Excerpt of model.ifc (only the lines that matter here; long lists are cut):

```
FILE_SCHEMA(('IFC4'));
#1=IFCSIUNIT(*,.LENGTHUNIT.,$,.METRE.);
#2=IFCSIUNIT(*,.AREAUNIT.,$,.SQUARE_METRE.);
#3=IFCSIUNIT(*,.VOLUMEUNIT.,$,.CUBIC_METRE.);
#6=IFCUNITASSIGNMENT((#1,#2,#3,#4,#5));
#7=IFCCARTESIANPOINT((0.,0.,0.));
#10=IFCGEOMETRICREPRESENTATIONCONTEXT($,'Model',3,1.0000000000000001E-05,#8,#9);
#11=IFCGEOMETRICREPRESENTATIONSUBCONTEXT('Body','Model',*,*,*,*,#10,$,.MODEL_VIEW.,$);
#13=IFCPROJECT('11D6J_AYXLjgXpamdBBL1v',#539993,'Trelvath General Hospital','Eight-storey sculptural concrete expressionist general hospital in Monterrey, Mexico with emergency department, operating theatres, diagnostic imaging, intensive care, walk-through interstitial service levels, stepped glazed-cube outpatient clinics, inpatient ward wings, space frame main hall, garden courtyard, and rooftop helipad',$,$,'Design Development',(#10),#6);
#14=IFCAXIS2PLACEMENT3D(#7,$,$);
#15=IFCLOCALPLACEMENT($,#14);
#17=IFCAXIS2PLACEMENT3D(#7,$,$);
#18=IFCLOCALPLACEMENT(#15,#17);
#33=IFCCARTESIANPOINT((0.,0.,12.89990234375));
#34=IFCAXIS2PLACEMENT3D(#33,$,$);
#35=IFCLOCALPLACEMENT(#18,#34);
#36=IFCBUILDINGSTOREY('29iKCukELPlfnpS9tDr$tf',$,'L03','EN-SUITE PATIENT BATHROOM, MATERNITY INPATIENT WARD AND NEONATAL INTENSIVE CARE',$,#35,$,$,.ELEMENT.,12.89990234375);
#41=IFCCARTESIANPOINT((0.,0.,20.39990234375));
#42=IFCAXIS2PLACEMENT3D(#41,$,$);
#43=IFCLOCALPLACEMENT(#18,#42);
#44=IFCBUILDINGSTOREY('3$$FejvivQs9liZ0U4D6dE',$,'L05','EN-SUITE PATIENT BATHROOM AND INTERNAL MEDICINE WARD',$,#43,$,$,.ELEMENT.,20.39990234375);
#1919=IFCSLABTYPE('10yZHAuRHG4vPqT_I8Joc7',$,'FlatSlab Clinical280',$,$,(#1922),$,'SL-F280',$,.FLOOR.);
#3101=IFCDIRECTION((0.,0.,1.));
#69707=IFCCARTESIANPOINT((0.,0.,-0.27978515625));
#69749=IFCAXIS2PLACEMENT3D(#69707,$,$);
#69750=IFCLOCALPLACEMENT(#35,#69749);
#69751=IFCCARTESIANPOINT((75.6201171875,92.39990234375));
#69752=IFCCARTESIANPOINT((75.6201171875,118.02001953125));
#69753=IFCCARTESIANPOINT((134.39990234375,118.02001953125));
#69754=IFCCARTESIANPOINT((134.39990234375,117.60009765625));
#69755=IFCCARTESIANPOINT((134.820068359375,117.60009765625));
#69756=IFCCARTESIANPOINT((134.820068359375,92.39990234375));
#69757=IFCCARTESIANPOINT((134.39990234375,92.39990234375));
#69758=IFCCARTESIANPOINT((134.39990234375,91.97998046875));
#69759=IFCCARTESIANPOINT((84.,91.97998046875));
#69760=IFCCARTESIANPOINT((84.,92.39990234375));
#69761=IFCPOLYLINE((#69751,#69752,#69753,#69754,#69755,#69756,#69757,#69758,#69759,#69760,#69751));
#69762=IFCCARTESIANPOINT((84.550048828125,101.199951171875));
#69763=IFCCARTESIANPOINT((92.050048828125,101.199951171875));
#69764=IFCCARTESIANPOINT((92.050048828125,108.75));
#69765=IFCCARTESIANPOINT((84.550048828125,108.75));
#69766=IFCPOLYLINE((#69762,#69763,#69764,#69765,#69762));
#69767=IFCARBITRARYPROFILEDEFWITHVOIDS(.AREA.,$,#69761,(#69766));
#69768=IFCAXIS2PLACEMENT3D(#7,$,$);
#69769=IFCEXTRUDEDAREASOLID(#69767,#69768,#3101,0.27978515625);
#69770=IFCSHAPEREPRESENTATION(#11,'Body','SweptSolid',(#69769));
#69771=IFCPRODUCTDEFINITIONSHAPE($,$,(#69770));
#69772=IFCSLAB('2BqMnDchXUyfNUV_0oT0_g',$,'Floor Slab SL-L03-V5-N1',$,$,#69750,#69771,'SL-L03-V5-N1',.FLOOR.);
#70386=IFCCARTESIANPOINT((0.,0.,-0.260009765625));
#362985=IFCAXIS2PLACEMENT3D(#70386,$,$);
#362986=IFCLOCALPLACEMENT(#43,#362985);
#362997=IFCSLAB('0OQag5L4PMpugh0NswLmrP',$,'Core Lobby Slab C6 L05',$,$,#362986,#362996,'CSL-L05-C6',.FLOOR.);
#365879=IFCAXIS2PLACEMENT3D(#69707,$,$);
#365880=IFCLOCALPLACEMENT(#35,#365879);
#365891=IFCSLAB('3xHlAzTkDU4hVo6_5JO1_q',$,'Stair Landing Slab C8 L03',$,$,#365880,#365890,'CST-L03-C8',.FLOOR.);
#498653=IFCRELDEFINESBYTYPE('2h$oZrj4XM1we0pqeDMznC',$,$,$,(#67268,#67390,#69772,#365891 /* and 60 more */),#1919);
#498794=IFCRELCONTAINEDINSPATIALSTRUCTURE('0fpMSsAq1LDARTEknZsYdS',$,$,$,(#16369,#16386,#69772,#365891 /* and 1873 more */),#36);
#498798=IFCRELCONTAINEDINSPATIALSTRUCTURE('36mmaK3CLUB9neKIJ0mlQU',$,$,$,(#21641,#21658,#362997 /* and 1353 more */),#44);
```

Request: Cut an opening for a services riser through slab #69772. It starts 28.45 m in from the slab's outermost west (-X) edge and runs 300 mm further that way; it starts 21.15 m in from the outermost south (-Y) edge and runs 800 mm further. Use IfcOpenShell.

```python
import numpy as np
import ifcopenshell
import ifcopenshell.api.feature
import ifcopenshell.api.geometry
import ifcopenshell.api.root
import ifcopenshell.geom
import ifcopenshell.util.placement
import ifcopenshell.util.representation
import ifcopenshell.util.shape
import ifcopenshell.util.unit

model = ifcopenshell.open("model.ifc")
unit_scale = ifcopenshell.util.unit.calculate_unit_scale(model)
settings = ifcopenshell.geom.settings()


def volume(element):
    """Net volume in cubic metres, openings subtracted."""
    shape = ifcopenshell.geom.create_shape(settings, element)
    return ifcopenshell.util.shape.get_volume(shape.geometry)


slab = model.by_guid("2BqMnDchXUyfNUV_0oT0_g")
before = volume(slab)

# Extent in the slab's own axes, in metres. The edges named are its -X and -Y sides.
slab_shape = ifcopenshell.geom.create_shape(settings, slab)
vertices = ifcopenshell.util.shape.get_vertices(slab_shape.geometry)
x_min, y_min, bottom = vertices.min(axis=0)
top = vertices[:, 2].max()

opening = ifcopenshell.api.root.create_entity(model, ifc_class="IfcOpeningElement", name="Services riser opening", predefined_type="OPENING")
context = ifcopenshell.util.representation.get_context(model, "Model", "Body", "MODEL_VIEW")
width, depth = 0.3, 0.8
outline = [(0.0, 0.0), (width, 0.0), (width, depth), (0.0, depth), (0.0, 0.0)]
# Overshoot both faces by 50 mm so the cut is clean.
shape = ifcopenshell.api.geometry.add_slab_representation(
    model, context=context, depth=top - bottom + 0.1, polyline=outline
)
ifcopenshell.api.geometry.assign_representation(model, product=opening, representation=shape)

matrix = ifcopenshell.util.placement.get_local_placement(slab.ObjectPlacement)
matrix[:, 3] = matrix @ np.append(np.array([x_min + 28.45, y_min + 21.15, bottom - 0.05]) / unit_scale, 1.0)
ifcopenshell.api.geometry.edit_object_placement(model, product=opening, matrix=matrix, is_si=False)
ifcopenshell.api.feature.add_feature(model, feature=opening, element=slab)

after = volume(slab)

print(f"slab volume {before:.3f} -> {after:.3f} m3")

model.write("model_rev.ifc")
```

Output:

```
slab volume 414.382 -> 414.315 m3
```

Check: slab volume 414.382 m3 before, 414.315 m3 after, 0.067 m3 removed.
